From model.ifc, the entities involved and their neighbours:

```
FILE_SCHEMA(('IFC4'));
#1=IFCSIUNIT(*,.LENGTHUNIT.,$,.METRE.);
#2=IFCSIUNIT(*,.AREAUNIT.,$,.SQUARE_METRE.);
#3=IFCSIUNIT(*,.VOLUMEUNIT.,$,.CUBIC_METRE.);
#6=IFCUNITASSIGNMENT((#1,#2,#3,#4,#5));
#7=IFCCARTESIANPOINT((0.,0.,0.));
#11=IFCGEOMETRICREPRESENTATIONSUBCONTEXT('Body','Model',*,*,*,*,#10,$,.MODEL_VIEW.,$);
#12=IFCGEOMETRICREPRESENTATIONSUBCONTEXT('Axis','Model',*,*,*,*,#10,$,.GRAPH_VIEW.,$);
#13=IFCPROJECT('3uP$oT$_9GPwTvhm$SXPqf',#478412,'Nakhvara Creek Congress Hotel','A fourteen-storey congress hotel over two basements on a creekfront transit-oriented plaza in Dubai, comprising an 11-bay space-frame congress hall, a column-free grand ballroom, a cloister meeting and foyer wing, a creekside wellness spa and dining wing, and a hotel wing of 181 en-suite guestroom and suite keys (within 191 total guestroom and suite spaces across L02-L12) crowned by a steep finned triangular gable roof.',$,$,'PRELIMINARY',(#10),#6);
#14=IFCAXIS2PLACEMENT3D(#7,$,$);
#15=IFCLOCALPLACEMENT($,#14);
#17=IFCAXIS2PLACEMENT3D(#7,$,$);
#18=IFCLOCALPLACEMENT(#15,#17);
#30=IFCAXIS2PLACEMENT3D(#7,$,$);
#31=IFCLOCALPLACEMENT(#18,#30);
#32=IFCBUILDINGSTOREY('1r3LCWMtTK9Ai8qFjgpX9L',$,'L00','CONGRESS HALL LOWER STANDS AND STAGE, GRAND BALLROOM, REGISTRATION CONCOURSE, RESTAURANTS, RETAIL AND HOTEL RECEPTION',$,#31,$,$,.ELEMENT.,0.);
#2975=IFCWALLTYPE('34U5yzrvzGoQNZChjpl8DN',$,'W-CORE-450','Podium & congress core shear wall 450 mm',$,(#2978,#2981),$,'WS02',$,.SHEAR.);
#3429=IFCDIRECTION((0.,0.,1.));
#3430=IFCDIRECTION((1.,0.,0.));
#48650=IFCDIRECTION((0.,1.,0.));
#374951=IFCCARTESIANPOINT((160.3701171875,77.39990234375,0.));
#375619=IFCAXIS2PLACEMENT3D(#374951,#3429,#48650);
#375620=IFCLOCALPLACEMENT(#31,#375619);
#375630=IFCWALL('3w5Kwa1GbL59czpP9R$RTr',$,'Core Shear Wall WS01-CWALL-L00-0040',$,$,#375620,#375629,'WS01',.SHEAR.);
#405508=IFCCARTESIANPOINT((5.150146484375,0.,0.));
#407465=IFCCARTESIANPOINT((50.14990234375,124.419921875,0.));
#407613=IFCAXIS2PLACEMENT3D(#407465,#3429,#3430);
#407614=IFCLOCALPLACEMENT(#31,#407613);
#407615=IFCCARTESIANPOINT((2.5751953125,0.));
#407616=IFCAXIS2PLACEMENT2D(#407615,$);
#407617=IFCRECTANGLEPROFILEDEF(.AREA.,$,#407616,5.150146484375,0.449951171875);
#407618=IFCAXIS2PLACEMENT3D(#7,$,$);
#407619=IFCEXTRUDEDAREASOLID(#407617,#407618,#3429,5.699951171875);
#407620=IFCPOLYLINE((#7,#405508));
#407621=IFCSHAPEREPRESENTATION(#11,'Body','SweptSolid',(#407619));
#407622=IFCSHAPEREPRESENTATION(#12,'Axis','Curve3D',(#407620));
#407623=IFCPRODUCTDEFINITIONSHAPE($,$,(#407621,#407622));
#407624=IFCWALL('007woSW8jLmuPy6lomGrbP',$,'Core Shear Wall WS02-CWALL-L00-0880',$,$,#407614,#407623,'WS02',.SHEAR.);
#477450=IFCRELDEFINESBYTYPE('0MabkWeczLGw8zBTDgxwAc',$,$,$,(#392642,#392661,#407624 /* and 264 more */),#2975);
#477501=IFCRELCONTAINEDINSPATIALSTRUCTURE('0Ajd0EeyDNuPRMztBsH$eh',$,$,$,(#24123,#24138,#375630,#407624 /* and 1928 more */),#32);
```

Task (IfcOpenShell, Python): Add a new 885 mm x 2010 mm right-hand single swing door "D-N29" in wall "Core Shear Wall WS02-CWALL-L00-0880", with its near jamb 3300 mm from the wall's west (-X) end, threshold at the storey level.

```python
import numpy as np
import ifcopenshell
import ifcopenshell.api.feature
import ifcopenshell.api.geometry
import ifcopenshell.api.root
import ifcopenshell.api.spatial
import ifcopenshell.geom
import ifcopenshell.util.element
import ifcopenshell.util.placement
import ifcopenshell.util.representation
import ifcopenshell.util.shape
import ifcopenshell.util.unit

model = ifcopenshell.open("model.ifc")
unit_scale = ifcopenshell.util.unit.calculate_unit_scale(model)
settings = ifcopenshell.geom.settings()


def volume(element):
    """Net volume in cubic metres, openings subtracted."""
    shape = ifcopenshell.geom.create_shape(settings, element)
    return ifcopenshell.util.shape.get_volume(shape.geometry)


wall = model.by_id(407624)
storey = ifcopenshell.util.element.get_container(wall, ifc_class="IfcBuildingStorey")
context = ifcopenshell.util.representation.get_context(model, "Model", "Body", "MODEL_VIEW")
before = volume(wall)

width, height, from_end, sill = 0.885, 2.01, 3.3, 0.0  # metres

# The wall runs along its own X axis, and the end named is its -X end.
wall_shape = ifcopenshell.geom.create_shape(settings, wall)
x, y, z = ifcopenshell.util.shape.get_vertices(wall_shape.geometry).T
start = x.min() + from_end
face, thickness = float(y.min()), float(y.max() - y.min())
wall_matrix = ifcopenshell.util.placement.get_local_placement(wall.ObjectPlacement)
level = ifcopenshell.util.placement.get_local_placement(storey.ObjectPlacement)[2, 3]


def in_wall(x, y):
    """Placement at x, y metres in the wall's axes, at sill height."""
    matrix = wall_matrix.copy()
    matrix[:, 3] = wall_matrix @ np.array([x / unit_scale, y / unit_scale, 0.0, 1.0])
    matrix[2, 3] = level + sill / unit_scale
    return matrix


# Opening: a box that overshoots both wall faces by 50 mm.
opening = ifcopenshell.api.root.create_entity(model, ifc_class="IfcOpeningElement", predefined_type="OPENING")
box = ifcopenshell.api.geometry.add_wall_representation(
    model, context=context, length=width, height=height, thickness=thickness + 0.1
)
ifcopenshell.api.geometry.assign_representation(model, product=opening, representation=box)
ifcopenshell.api.geometry.edit_object_placement(model, product=opening, matrix=in_wall(start, face - 0.05), is_si=False)
ifcopenshell.api.feature.add_feature(model, feature=opening, element=wall)

door = ifcopenshell.api.root.create_entity(model, ifc_class="IfcDoor", name="D-N29", predefined_type="DOOR")
door.OverallWidth, door.OverallHeight = width / unit_scale, height / unit_scale
door.OperationType = "SINGLE_SWING_RIGHT"
body = ifcopenshell.api.geometry.add_door_representation(
    model,
    context=context,
    overall_width=door.OverallWidth,
    overall_height=door.OverallHeight,
    operation_type="SINGLE_SWING_RIGHT",
    lining_properties={"LiningDepth": thickness / unit_scale, "ThresholdDepth": thickness / unit_scale},
)
ifcopenshell.api.geometry.assign_representation(model, product=door, representation=body)
ifcopenshell.api.spatial.assign_container(model, products=[door], relating_structure=storey)
ifcopenshell.api.feature.add_filling(model, opening=opening, element=door)

# The lining spans the wall, so the door starts at the wall face.
ifcopenshell.api.geometry.edit_object_placement(model, product=door, matrix=in_wall(start, face), is_si=False)

after = volume(wall)

print(f"wall volume {before:.3f} -> {after:.3f} m3")

model.write("model_v2.ifc")
```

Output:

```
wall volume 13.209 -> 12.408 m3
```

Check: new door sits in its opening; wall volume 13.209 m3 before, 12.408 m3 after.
